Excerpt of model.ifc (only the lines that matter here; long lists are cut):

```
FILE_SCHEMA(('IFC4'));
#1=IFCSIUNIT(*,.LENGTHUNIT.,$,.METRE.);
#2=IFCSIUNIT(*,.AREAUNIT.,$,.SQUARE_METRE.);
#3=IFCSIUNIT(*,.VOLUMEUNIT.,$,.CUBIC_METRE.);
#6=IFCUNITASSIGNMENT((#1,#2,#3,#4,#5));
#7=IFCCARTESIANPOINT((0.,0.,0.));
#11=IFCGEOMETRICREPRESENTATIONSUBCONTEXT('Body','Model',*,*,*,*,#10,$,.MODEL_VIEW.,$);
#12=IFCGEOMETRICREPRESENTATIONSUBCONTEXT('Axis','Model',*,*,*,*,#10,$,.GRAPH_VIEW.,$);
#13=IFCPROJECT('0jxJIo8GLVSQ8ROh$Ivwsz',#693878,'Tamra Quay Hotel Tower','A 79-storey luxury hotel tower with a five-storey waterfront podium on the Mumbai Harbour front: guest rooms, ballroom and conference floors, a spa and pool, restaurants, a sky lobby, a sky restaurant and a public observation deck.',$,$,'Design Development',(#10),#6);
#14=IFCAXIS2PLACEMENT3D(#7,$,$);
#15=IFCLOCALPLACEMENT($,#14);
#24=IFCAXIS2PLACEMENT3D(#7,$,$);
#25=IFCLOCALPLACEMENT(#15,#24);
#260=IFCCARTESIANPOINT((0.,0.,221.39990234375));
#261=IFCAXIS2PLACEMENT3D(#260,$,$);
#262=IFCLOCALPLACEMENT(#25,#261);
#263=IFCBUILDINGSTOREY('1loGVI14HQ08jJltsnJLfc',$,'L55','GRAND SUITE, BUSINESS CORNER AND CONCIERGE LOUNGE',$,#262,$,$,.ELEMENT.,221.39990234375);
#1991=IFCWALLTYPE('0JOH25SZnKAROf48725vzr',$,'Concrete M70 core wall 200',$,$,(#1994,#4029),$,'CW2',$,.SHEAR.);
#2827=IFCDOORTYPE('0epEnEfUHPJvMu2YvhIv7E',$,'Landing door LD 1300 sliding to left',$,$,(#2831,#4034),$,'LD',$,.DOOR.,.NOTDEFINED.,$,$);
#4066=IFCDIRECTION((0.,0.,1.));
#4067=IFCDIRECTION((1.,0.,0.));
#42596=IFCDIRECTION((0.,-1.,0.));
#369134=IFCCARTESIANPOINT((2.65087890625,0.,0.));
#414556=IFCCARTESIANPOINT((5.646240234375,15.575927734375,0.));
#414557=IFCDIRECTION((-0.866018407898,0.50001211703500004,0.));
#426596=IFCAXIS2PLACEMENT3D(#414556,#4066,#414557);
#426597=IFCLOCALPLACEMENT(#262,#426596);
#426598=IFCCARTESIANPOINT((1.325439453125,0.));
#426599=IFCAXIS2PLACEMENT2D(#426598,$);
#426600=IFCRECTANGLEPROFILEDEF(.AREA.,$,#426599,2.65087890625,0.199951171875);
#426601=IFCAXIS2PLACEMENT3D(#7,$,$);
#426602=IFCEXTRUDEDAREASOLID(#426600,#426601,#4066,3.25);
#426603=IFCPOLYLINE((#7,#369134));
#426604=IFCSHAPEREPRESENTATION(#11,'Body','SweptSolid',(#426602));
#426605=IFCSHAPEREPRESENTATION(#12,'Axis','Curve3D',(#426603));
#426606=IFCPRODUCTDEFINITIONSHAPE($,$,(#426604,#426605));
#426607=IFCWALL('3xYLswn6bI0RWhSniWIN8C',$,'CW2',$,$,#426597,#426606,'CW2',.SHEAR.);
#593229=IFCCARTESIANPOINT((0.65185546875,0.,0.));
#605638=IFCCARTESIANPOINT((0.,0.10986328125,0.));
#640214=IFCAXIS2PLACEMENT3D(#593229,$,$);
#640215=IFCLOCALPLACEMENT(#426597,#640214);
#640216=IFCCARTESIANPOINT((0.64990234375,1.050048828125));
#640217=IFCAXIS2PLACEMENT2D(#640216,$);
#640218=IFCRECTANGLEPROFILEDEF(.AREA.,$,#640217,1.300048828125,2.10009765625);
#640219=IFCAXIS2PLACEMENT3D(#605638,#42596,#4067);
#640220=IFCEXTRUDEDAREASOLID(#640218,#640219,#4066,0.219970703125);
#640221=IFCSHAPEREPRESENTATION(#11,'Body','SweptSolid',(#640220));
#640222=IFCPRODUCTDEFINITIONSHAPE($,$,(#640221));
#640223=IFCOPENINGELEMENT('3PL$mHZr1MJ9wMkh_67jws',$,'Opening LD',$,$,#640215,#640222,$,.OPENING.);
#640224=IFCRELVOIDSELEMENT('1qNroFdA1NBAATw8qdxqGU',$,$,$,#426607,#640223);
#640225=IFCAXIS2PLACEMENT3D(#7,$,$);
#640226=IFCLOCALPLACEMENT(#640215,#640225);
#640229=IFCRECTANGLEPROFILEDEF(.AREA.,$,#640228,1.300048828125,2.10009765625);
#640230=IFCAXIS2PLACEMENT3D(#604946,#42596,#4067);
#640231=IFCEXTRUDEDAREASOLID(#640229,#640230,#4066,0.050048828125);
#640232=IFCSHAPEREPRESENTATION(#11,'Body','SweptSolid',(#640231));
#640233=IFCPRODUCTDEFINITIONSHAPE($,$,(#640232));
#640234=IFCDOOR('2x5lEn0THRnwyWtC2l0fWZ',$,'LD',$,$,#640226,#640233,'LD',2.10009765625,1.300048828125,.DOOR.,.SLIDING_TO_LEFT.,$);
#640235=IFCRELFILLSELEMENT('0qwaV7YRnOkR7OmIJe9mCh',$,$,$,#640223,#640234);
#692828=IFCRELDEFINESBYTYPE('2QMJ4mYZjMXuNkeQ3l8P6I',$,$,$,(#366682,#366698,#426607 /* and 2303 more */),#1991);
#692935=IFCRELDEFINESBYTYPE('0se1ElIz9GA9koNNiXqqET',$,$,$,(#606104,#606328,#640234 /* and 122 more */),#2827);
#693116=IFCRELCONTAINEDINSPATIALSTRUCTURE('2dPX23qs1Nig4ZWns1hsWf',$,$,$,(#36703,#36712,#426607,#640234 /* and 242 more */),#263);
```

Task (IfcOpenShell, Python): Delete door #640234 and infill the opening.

```python
import ifcopenshell
import ifcopenshell.api.feature
import ifcopenshell.api.root
import ifcopenshell.geom
import ifcopenshell.util.shape

model = ifcopenshell.open("model.ifc")
settings = ifcopenshell.geom.settings()


def volume(element):
    """Net volume in cubic metres, openings subtracted."""
    shape = ifcopenshell.geom.create_shape(settings, element)
    return ifcopenshell.util.shape.get_volume(shape.geometry)


door = model.by_id(640234)
opening = door.FillsVoids[0].RelatingOpeningElement
wall = opening.VoidsElements[0].RelatingBuildingElement
before = volume(wall)

ifcopenshell.api.root.remove_product(model, product=door)
ifcopenshell.api.feature.remove_feature(model, feature=opening)

after = volume(wall)

print(f"wall volume {before:.3f} -> {after:.3f} m3")

model.write("model_v2.ifc")
```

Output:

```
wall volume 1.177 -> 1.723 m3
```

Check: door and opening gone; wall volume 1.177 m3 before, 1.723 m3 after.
